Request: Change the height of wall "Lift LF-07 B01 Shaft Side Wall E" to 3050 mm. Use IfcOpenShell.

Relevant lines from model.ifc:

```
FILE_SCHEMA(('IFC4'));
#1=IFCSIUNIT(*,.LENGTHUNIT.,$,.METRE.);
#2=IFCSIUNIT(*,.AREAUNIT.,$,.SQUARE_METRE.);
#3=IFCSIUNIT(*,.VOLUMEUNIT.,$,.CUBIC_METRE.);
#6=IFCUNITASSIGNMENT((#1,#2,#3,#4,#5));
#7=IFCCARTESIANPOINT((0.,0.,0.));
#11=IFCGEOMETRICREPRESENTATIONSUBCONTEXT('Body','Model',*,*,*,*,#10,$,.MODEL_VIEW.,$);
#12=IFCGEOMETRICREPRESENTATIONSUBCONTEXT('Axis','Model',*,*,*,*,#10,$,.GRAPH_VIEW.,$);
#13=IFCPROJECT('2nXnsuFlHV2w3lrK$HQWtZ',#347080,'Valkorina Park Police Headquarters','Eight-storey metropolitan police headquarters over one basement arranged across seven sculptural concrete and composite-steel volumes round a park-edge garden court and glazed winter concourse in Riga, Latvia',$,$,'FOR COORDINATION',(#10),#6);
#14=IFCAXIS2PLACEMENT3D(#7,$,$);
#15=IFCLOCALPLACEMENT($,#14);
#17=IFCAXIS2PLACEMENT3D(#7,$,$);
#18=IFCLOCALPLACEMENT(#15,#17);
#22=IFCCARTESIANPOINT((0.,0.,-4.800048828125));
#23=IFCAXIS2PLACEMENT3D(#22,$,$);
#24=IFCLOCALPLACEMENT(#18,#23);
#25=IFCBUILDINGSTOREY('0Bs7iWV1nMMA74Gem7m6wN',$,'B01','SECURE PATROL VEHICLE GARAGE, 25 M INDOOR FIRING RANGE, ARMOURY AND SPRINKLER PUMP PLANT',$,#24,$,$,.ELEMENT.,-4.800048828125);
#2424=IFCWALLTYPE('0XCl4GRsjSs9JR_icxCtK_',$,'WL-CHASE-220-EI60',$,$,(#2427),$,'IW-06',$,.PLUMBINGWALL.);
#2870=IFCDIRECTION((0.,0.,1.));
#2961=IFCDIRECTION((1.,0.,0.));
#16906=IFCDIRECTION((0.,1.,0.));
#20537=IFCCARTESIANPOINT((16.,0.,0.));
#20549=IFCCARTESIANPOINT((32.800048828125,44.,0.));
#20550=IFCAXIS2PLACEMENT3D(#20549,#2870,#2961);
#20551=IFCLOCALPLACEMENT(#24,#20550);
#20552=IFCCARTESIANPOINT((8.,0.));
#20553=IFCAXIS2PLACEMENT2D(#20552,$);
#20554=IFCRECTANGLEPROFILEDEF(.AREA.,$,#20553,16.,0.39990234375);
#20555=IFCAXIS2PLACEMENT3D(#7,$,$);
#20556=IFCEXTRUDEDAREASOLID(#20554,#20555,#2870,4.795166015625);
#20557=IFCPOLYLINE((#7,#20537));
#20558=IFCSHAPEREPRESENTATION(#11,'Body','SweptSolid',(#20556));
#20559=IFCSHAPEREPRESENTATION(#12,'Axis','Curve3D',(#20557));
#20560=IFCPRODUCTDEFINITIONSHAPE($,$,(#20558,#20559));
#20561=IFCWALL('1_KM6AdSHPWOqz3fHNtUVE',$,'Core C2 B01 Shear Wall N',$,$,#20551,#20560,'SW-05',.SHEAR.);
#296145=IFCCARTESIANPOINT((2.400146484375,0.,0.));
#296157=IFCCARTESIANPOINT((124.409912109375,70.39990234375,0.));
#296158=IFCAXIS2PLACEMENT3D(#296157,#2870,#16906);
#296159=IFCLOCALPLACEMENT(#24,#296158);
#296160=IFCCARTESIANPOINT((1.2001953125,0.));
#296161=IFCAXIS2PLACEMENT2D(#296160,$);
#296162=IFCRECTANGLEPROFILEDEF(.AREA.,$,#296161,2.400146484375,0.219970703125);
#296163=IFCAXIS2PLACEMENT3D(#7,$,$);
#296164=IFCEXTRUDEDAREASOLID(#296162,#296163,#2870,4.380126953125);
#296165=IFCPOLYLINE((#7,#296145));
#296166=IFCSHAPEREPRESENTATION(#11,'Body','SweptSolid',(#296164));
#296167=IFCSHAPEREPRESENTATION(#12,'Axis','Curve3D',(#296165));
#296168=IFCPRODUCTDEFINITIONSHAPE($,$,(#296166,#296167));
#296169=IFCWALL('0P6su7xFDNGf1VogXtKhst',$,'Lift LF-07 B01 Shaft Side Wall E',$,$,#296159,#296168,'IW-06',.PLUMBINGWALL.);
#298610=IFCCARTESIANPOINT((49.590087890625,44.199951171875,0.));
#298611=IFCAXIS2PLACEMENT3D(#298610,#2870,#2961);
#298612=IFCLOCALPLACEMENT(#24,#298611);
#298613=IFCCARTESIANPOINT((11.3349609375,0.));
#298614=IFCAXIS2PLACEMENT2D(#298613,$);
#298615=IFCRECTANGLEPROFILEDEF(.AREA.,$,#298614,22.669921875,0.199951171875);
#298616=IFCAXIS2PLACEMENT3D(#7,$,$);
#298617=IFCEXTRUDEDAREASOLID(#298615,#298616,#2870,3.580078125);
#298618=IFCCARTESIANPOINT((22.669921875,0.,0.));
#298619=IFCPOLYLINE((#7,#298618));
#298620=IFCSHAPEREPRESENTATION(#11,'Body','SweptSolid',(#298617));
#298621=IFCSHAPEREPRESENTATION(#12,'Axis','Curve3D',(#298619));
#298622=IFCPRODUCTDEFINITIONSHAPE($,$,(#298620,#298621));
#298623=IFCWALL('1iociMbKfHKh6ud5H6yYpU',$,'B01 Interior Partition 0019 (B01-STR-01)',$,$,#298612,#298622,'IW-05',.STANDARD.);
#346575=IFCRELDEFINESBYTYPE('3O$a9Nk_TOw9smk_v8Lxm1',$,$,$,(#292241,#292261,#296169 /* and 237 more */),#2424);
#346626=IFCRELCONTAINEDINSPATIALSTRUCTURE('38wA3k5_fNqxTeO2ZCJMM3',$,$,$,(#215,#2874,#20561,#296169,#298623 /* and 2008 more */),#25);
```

```python
import ifcopenshell
import ifcopenshell.geom
import ifcopenshell.util.representation
import ifcopenshell.util.shape
import ifcopenshell.util.unit

model = ifcopenshell.open("model.ifc")
unit_scale = ifcopenshell.util.unit.calculate_unit_scale(model)
settings = ifcopenshell.geom.settings()


def volume(element):
    """Net volume in cubic metres, openings subtracted."""
    shape = ifcopenshell.geom.create_shape(settings, element)
    return ifcopenshell.util.shape.get_volume(shape.geometry)


wall = model.by_guid("0P6su7xFDNGf1VogXtKhst")
before = volume(wall)

body = ifcopenshell.util.representation.get_representation(wall, "Model", "Body")
solid = body.Items[0]
old_height = solid.Depth
solid.Depth = 3.05 / unit_scale
after = volume(wall)

print(f"height {old_height:g} -> {solid.Depth:g}, volume {before:.3f} -> {after:.3f} m3")

model.write("model_v2.ifc")
```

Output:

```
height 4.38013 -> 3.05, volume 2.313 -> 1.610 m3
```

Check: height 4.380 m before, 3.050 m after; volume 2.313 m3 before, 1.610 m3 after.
